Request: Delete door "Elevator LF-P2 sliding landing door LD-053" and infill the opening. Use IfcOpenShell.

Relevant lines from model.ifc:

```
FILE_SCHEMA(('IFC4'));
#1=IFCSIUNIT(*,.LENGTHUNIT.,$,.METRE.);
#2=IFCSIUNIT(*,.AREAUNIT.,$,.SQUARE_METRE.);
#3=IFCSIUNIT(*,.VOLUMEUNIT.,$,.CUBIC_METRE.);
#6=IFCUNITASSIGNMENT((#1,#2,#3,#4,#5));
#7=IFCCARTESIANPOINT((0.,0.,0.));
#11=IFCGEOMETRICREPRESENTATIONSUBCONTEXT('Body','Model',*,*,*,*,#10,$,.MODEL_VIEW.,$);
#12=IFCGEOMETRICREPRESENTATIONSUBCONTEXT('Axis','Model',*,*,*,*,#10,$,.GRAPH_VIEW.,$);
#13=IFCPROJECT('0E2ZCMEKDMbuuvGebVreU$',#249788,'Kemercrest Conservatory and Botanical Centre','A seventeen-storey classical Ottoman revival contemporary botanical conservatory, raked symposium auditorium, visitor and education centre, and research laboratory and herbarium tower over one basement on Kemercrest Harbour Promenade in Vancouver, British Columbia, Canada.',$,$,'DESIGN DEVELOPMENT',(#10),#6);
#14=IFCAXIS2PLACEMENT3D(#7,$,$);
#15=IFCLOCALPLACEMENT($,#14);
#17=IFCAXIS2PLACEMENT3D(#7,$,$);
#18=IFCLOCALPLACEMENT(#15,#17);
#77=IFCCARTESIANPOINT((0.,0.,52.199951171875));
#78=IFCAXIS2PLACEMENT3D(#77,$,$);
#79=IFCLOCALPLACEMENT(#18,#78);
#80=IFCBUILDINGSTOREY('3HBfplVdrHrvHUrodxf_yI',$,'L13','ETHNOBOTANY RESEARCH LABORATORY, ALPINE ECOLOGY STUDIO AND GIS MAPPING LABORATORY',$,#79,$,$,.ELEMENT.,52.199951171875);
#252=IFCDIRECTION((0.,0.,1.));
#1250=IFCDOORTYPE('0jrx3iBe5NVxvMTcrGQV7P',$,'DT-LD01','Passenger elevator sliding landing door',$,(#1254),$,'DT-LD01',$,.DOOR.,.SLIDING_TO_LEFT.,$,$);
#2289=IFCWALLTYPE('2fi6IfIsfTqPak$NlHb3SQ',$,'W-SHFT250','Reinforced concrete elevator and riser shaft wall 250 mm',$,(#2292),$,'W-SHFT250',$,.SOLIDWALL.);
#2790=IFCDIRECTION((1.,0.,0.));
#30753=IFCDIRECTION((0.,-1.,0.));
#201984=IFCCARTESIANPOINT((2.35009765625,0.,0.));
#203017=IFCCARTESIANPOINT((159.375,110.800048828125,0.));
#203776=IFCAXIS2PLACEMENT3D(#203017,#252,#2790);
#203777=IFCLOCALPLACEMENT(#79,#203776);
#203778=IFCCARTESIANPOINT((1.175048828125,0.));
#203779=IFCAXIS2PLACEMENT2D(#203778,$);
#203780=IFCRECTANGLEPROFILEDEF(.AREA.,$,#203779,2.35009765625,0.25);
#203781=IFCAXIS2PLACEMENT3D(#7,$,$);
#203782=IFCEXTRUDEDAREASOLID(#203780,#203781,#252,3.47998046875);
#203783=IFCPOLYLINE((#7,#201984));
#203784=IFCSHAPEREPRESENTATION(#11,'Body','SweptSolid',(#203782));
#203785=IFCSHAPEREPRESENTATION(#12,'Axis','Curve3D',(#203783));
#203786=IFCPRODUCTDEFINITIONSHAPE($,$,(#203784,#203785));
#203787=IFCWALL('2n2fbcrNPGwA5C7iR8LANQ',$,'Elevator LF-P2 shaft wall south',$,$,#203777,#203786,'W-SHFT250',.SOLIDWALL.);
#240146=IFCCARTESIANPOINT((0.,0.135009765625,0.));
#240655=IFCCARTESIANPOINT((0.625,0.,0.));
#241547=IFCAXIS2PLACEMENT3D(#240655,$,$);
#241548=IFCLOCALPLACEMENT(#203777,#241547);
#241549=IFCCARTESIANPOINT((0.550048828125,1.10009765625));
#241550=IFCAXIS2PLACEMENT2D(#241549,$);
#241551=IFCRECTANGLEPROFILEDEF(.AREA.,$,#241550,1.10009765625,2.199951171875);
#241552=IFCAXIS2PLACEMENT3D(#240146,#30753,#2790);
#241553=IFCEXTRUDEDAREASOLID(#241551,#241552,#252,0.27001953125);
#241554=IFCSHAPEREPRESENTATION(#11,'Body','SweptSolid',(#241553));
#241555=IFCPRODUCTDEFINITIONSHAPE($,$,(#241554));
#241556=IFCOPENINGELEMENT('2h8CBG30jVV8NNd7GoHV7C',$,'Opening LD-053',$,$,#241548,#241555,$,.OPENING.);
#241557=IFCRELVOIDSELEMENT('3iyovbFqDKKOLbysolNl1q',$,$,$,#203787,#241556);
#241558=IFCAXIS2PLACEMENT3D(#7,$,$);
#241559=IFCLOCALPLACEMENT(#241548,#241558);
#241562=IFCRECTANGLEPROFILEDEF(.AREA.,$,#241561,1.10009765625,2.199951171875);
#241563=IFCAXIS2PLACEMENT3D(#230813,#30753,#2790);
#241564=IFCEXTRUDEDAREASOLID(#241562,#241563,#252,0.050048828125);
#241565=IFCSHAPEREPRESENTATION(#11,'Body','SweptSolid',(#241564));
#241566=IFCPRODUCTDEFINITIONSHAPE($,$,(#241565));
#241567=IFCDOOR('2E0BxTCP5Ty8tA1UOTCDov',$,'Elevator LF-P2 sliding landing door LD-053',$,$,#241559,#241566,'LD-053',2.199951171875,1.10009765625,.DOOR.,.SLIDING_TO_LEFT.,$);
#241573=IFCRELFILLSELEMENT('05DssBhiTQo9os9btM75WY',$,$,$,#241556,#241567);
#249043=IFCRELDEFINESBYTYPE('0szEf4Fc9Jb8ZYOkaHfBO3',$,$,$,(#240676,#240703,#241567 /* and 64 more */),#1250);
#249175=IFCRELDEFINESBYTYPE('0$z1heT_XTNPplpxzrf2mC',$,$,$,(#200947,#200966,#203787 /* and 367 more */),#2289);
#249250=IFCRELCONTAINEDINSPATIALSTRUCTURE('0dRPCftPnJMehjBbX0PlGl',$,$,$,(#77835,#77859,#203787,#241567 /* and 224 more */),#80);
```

```python
import ifcopenshell
import ifcopenshell.api.feature
import ifcopenshell.api.root
import ifcopenshell.geom
import ifcopenshell.util.shape

model = ifcopenshell.open("model.ifc")
settings = ifcopenshell.geom.settings()


def volume(element):
    """Net volume in cubic metres, openings subtracted."""
    shape = ifcopenshell.geom.create_shape(settings, element)
    return ifcopenshell.util.shape.get_volume(shape.geometry)


door = model.by_id(241567)
opening = door.FillsVoids[0].RelatingOpeningElement
wall = opening.VoidsElements[0].RelatingBuildingElement
before = volume(wall)

ifcopenshell.api.root.remove_product(model, product=door)
ifcopenshell.api.feature.remove_feature(model, feature=opening)

after = volume(wall)

print(f"wall volume {before:.3f} -> {after:.3f} m3")

model.write("model_rev.ifc")
```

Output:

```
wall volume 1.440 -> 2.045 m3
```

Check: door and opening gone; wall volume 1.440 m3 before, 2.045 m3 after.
